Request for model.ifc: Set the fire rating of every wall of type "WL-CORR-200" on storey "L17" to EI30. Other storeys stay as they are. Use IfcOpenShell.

First a look at what the model holds.

```python
import ifcopenshell
import ifcopenshell.util.element

model = ifcopenshell.open("model.ifc")
print(model.schema)
storey = next(s for s in model.by_type("IfcBuildingStorey") if s.Name == "L17")
walls = [e for e in ifcopenshell.util.element.get_decomposition(storey) if e.is_a("IfcWall")]
seen = {}
for e in walls:
    element_type = ifcopenshell.util.element.get_type(e)
    key = (element_type.Name if element_type != e and element_type else None, ifcopenshell.util.element.get_pset(e, "Pset_WallCommon", "FireRating"))
    seen[key] = seen.get(key, 0) + 1
for (name, value), count in sorted(seen.items(), key=str):
    print(count, "x", name, "|", value)
```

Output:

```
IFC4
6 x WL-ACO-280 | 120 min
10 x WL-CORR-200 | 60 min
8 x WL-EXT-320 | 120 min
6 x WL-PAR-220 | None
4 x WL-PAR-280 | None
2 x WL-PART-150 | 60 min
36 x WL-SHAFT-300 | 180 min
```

```python
import ifcopenshell
import ifcopenshell.api.pset
import ifcopenshell.util.element

model = ifcopenshell.open("model.ifc")

storey = next(s for s in model.by_type("IfcBuildingStorey") if s.Name == "L17")
walls = [e for e in ifcopenshell.util.element.get_decomposition(storey) if e.is_a("IfcWall")]

count = 0
for e in walls:
    element_type = ifcopenshell.util.element.get_type(e)
    if element_type in (None, e) or element_type.Name != "WL-CORR-200":
        continue
    # add_pset returns the element's existing set when there is one.
    pset = ifcopenshell.api.pset.add_pset(model, product=e, name="Pset_WallCommon")
    ifcopenshell.api.pset.edit_pset(model, pset=pset, properties={"FireRating": "EI30"})
    count += 1

print(count, "walls updated")

model.write("model_updated.ifc")
```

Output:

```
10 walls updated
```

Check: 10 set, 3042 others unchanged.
